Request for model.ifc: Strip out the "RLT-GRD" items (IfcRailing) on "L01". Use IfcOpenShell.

First a look at what the model holds.

```python
import ifcopenshell
import ifcopenshell.util.element

model = ifcopenshell.open("model.ifc")
print(model.schema)
storey = next(s for s in model.by_type("IfcBuildingStorey") if s.Name == "L01")
railings = [e for e in ifcopenshell.util.element.get_decomposition(storey) if e.is_a("IfcRailing")]
seen = {}
for e in railings:
    element_type = ifcopenshell.util.element.get_type(e)
    name = element_type.Name if element_type not in (None, e) else None
    seen[name] = seen.get(name, 0) + 1
for name, count in sorted(seen.items(), key=str):
    print(count, "x", name)
```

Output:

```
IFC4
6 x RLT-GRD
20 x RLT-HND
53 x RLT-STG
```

```python
import ifcopenshell
import ifcopenshell.api.root
import ifcopenshell.util.element

model = ifcopenshell.open("model.ifc")

storey = next(s for s in model.by_type("IfcBuildingStorey") if s.Name == "L01")
railings = [e for e in ifcopenshell.util.element.get_decomposition(storey) if e.is_a("IfcRailing")]
targets = [e for e in railings if (t := ifcopenshell.util.element.get_type(e)) not in (None, e) and t.Name == "RLT-GRD"]

for e in targets:
    ifcopenshell.api.root.remove_product(model, product=e)
print(len(targets), "removed")

model.write("model_rev.ifc")
```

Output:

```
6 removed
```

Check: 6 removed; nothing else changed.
